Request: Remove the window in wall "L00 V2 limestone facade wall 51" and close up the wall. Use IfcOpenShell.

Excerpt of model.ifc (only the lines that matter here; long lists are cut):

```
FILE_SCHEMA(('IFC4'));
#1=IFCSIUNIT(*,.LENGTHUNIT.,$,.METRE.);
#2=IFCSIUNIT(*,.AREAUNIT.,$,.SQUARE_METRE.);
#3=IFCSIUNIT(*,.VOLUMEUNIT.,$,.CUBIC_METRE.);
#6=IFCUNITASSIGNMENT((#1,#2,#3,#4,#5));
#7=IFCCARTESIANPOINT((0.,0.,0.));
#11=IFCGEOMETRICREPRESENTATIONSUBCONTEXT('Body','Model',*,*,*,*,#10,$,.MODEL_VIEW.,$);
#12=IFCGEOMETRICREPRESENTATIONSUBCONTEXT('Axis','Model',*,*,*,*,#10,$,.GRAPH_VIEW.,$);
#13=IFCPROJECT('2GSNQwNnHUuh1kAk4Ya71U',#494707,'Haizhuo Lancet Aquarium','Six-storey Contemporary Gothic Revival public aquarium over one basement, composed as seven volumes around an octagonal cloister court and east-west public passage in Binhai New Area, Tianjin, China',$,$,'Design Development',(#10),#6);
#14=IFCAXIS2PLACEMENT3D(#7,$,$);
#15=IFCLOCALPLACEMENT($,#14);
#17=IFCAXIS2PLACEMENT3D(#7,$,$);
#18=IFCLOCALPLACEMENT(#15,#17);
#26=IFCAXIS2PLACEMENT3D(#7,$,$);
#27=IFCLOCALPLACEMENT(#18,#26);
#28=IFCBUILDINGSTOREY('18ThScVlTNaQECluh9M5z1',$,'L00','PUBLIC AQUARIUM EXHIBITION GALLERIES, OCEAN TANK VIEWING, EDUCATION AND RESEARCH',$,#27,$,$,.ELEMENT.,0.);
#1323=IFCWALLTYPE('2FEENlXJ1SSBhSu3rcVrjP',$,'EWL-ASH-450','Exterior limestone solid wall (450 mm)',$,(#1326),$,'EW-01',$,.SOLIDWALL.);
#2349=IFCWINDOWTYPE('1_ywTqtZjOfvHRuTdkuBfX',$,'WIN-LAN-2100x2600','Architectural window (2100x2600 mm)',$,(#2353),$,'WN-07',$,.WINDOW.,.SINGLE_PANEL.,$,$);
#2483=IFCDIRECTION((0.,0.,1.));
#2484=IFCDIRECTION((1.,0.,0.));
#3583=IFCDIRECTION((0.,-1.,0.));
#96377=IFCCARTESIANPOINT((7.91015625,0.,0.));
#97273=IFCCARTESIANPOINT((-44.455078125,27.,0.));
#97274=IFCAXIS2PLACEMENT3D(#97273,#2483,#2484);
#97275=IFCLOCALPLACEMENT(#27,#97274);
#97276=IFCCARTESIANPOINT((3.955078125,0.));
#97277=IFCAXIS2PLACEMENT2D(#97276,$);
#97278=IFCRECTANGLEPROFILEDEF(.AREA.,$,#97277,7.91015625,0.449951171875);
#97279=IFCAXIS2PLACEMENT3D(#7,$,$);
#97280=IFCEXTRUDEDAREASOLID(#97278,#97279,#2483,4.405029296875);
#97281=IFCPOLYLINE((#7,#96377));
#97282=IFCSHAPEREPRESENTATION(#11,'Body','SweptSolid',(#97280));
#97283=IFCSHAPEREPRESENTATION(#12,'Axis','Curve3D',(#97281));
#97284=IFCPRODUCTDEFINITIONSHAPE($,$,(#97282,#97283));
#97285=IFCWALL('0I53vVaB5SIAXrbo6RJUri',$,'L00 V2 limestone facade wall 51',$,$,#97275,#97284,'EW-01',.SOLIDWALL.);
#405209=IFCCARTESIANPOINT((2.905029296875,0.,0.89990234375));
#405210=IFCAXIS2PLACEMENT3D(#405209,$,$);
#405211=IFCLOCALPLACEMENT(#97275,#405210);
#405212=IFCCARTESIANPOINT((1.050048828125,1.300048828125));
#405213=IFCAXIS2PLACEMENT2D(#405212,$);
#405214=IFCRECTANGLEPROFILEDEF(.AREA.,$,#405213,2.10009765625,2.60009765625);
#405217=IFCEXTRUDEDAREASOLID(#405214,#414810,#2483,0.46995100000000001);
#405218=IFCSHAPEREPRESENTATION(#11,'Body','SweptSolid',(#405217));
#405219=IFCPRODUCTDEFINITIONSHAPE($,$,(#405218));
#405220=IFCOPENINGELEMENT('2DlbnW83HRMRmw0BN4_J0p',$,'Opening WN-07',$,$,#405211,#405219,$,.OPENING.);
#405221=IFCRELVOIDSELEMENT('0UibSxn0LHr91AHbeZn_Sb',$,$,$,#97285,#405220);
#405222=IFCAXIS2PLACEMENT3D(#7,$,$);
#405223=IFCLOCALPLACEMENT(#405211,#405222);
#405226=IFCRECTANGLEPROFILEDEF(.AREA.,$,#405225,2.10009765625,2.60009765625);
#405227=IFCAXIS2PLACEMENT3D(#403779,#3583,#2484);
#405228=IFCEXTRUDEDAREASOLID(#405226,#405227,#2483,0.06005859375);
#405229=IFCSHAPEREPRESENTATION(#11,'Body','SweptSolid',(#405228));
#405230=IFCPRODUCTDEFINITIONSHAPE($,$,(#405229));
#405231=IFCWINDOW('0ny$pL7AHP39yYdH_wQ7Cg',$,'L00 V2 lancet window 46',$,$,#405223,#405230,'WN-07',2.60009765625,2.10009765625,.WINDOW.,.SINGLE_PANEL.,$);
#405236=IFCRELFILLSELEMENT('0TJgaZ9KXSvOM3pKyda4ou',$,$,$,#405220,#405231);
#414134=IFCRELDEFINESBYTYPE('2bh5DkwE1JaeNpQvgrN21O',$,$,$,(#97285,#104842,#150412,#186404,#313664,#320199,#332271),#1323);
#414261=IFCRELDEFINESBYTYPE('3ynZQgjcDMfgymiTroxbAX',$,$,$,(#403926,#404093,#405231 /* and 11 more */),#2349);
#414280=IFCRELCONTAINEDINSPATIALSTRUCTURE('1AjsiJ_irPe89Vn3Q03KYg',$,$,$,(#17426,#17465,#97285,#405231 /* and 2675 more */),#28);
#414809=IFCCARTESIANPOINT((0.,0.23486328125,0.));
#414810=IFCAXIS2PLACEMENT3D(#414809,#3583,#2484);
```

```python
import ifcopenshell
import ifcopenshell.api.feature
import ifcopenshell.api.root
import ifcopenshell.geom
import ifcopenshell.util.shape

model = ifcopenshell.open("model.ifc")
settings = ifcopenshell.geom.settings()


def volume(element):
    """Net volume in cubic metres, openings subtracted."""
    shape = ifcopenshell.geom.create_shape(settings, element)
    return ifcopenshell.util.shape.get_volume(shape.geometry)


window = model.by_guid("0ny$pL7AHP39yYdH_wQ7Cg")
opening = window.FillsVoids[0].RelatingOpeningElement
wall = opening.VoidsElements[0].RelatingBuildingElement
before = volume(wall)

ifcopenshell.api.root.remove_product(model, product=window)
ifcopenshell.api.feature.remove_feature(model, feature=opening)

after = volume(wall)

print(f"wall volume {before:.3f} -> {after:.3f} m3")

model.write("model_edited.ifc")
```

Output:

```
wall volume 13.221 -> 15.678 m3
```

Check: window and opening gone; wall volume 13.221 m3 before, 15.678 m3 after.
